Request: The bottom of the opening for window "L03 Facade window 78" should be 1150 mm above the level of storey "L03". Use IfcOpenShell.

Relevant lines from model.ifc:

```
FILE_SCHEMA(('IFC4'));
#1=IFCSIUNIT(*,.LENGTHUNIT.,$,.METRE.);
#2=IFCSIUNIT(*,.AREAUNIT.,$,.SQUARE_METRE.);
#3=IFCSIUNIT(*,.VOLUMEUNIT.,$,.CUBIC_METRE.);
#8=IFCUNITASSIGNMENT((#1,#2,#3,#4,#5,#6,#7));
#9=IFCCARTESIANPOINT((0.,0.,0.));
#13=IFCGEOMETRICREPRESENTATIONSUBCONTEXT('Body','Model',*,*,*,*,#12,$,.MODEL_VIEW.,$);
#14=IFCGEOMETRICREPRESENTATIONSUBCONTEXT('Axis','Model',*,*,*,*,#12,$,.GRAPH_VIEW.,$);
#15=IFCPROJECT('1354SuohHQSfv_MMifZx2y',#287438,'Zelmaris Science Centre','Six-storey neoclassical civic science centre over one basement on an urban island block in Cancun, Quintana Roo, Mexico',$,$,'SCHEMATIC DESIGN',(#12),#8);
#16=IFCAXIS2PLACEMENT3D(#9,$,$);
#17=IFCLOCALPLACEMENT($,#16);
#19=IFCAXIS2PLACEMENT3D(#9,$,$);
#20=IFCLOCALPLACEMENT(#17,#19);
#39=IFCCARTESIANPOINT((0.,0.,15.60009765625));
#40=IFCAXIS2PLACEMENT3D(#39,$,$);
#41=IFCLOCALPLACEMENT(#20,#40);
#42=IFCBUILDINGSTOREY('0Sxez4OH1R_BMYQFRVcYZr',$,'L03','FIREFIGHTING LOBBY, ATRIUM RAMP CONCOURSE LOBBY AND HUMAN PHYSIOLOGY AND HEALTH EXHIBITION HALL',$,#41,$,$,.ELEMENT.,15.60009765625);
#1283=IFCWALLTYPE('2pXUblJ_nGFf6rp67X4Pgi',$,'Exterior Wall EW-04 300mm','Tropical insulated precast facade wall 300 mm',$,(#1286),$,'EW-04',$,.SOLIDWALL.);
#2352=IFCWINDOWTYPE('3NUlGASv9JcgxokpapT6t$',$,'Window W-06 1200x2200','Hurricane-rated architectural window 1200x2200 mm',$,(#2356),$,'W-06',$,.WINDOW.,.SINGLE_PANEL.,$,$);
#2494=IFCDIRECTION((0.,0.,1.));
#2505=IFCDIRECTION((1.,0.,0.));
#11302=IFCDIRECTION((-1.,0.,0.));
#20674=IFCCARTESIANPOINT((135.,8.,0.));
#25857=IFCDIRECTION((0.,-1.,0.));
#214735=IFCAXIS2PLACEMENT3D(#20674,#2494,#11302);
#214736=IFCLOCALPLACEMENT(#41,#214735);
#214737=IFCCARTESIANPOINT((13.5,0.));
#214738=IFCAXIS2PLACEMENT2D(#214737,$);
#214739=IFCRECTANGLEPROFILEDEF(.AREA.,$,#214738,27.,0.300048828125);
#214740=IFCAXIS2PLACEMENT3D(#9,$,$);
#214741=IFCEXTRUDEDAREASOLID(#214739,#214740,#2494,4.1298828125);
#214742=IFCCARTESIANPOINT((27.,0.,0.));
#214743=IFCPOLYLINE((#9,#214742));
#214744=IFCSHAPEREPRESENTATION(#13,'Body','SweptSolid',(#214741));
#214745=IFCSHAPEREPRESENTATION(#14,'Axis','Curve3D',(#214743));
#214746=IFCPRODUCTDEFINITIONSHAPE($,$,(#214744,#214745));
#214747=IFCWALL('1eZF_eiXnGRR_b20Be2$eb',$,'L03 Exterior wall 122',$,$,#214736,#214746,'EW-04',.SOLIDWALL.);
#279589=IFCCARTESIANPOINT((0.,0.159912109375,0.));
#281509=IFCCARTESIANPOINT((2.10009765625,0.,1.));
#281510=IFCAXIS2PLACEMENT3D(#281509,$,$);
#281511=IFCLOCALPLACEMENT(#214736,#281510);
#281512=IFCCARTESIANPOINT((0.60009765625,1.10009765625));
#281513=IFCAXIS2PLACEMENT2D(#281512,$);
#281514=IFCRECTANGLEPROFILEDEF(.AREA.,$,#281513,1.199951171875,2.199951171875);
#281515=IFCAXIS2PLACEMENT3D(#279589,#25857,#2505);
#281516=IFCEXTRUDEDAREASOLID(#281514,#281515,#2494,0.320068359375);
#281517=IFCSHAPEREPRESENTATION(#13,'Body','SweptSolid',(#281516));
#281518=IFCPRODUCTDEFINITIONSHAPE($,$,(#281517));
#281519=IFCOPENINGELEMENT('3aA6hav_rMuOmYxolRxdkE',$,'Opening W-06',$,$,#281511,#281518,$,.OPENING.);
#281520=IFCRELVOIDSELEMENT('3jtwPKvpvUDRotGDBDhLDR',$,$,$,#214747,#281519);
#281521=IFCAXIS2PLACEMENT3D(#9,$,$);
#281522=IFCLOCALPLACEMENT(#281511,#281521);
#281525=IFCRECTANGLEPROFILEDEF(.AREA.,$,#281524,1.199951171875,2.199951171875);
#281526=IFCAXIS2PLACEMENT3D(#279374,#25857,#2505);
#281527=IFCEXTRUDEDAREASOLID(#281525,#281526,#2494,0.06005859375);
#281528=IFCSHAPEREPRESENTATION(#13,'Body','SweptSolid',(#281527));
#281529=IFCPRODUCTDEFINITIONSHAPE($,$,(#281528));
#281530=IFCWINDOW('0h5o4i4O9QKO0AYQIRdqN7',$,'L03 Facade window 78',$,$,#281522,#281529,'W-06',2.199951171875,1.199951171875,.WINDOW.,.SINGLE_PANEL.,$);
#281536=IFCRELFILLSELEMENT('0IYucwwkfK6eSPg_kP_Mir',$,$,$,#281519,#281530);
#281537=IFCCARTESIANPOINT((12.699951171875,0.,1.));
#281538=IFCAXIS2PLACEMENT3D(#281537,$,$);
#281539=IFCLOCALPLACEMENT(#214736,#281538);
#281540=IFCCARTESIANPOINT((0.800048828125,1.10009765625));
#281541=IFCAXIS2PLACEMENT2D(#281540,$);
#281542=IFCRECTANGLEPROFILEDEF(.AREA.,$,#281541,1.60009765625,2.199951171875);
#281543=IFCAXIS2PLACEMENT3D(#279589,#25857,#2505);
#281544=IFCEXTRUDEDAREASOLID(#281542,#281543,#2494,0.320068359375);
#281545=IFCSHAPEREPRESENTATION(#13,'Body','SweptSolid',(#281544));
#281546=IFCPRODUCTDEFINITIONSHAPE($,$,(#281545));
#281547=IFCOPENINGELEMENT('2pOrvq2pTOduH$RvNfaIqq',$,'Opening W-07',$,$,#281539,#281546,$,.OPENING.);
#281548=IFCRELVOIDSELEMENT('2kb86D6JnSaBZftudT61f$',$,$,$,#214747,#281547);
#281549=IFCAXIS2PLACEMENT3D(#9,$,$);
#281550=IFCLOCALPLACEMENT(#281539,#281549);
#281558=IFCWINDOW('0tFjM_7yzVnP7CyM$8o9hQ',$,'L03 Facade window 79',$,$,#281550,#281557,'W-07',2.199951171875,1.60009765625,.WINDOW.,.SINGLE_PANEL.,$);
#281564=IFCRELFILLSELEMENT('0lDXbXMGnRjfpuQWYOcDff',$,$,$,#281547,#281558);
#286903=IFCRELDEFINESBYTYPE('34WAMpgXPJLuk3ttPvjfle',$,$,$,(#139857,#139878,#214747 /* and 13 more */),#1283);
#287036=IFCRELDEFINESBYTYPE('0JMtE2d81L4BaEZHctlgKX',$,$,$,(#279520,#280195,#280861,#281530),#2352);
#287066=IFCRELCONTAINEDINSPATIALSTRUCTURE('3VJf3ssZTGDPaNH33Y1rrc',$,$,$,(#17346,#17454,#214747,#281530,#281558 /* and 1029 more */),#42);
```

```python
import numpy as np
import ifcopenshell
import ifcopenshell.api.geometry
import ifcopenshell.geom
import ifcopenshell.util.element
import ifcopenshell.util.placement
import ifcopenshell.util.shape
import ifcopenshell.util.unit

model = ifcopenshell.open("model.ifc")
unit_scale = ifcopenshell.util.unit.calculate_unit_scale(model)

window = model.by_guid("0h5o4i4O9QKO0AYQIRdqN7")
opening = window.FillsVoids[0].RelatingOpeningElement
storey = ifcopenshell.util.element.get_container(window, ifc_class="IfcBuildingStorey")
level = ifcopenshell.util.placement.get_local_placement(storey.ObjectPlacement)[2, 3]

# The opening's origin need not be at the sill, so measure its lowest point.
shape = ifcopenshell.geom.create_shape(ifcopenshell.geom.settings(), opening)
bottom = ifcopenshell.util.shape.get_shape_bottom_elevation(shape, shape.geometry) / unit_scale
dz = level + 1.15 - bottom

shift = np.array([0.0, 0.0, dz])
# The window is placed relative to its opening, so it follows when the opening moves.
matrix = ifcopenshell.util.placement.get_local_placement(opening.ObjectPlacement)
matrix[:3, 3] += shift
ifcopenshell.api.geometry.edit_object_placement(
    model, product=opening, matrix=matrix, is_si=False, should_transform_children=True
)

print(f"moved by {dz * unit_scale:+.3f} m")

model.write("model_v2.ifc")
```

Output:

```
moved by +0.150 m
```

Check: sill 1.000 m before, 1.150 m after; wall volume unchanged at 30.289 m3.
